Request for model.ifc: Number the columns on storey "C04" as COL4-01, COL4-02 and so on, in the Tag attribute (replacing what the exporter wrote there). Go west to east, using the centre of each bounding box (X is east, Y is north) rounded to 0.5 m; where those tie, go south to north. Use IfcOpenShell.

First a look at what the model holds.

```python
import ifcopenshell
import ifcopenshell.util.element
import ifcopenshell.util.placement

model = ifcopenshell.open("model.ifc")
print(model.schema)
storey = next(s for s in model.by_type("IfcBuildingStorey") if s.Name == "C04")
columns = [e for e in ifcopenshell.util.element.get_decomposition(storey) if e.is_a("IfcColumn")]
for e in sorted(columns, key=lambda e: e.id()):
    origin = ifcopenshell.util.placement.get_local_placement(e.ObjectPlacement)[:3, 3]
    print(e.id(), e.Tag, e.Name, origin.round(2) + 0.0, sep=" | ")
```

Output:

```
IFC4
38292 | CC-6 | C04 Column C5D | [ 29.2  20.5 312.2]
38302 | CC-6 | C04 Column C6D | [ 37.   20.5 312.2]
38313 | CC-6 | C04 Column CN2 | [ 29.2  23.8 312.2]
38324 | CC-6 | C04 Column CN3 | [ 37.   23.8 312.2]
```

```python
import ifcopenshell
import ifcopenshell.geom
import ifcopenshell.util.element
import ifcopenshell.util.shape

model = ifcopenshell.open("model.ifc")
settings = ifcopenshell.geom.settings()
settings.set("use-world-coords", True)


def centre(element):
    shape = ifcopenshell.geom.create_shape(settings, element)
    return ifcopenshell.util.shape.get_bbox_centroid(shape.geometry)


storey = next(s for s in model.by_type("IfcBuildingStorey") if s.Name == "C04")
columns = [e for e in ifcopenshell.util.element.get_decomposition(storey) if e.is_a("IfcColumn")]

# Insertion points can sit at a corner or the storey origin, so sort by the geometry (in metres).
centres = {e: centre(e) for e in columns}
columns.sort(key=lambda e: (round(centres[e][0] / 0.5), centres[e][1]))

for i, e in enumerate(columns, start=1):
    number = f"COL4-{i:02d}"
    e.Tag = number
    print(e.id(), number)

model.write("model_edited.ifc")
```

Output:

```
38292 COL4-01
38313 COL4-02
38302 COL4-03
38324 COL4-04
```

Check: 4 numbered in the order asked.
